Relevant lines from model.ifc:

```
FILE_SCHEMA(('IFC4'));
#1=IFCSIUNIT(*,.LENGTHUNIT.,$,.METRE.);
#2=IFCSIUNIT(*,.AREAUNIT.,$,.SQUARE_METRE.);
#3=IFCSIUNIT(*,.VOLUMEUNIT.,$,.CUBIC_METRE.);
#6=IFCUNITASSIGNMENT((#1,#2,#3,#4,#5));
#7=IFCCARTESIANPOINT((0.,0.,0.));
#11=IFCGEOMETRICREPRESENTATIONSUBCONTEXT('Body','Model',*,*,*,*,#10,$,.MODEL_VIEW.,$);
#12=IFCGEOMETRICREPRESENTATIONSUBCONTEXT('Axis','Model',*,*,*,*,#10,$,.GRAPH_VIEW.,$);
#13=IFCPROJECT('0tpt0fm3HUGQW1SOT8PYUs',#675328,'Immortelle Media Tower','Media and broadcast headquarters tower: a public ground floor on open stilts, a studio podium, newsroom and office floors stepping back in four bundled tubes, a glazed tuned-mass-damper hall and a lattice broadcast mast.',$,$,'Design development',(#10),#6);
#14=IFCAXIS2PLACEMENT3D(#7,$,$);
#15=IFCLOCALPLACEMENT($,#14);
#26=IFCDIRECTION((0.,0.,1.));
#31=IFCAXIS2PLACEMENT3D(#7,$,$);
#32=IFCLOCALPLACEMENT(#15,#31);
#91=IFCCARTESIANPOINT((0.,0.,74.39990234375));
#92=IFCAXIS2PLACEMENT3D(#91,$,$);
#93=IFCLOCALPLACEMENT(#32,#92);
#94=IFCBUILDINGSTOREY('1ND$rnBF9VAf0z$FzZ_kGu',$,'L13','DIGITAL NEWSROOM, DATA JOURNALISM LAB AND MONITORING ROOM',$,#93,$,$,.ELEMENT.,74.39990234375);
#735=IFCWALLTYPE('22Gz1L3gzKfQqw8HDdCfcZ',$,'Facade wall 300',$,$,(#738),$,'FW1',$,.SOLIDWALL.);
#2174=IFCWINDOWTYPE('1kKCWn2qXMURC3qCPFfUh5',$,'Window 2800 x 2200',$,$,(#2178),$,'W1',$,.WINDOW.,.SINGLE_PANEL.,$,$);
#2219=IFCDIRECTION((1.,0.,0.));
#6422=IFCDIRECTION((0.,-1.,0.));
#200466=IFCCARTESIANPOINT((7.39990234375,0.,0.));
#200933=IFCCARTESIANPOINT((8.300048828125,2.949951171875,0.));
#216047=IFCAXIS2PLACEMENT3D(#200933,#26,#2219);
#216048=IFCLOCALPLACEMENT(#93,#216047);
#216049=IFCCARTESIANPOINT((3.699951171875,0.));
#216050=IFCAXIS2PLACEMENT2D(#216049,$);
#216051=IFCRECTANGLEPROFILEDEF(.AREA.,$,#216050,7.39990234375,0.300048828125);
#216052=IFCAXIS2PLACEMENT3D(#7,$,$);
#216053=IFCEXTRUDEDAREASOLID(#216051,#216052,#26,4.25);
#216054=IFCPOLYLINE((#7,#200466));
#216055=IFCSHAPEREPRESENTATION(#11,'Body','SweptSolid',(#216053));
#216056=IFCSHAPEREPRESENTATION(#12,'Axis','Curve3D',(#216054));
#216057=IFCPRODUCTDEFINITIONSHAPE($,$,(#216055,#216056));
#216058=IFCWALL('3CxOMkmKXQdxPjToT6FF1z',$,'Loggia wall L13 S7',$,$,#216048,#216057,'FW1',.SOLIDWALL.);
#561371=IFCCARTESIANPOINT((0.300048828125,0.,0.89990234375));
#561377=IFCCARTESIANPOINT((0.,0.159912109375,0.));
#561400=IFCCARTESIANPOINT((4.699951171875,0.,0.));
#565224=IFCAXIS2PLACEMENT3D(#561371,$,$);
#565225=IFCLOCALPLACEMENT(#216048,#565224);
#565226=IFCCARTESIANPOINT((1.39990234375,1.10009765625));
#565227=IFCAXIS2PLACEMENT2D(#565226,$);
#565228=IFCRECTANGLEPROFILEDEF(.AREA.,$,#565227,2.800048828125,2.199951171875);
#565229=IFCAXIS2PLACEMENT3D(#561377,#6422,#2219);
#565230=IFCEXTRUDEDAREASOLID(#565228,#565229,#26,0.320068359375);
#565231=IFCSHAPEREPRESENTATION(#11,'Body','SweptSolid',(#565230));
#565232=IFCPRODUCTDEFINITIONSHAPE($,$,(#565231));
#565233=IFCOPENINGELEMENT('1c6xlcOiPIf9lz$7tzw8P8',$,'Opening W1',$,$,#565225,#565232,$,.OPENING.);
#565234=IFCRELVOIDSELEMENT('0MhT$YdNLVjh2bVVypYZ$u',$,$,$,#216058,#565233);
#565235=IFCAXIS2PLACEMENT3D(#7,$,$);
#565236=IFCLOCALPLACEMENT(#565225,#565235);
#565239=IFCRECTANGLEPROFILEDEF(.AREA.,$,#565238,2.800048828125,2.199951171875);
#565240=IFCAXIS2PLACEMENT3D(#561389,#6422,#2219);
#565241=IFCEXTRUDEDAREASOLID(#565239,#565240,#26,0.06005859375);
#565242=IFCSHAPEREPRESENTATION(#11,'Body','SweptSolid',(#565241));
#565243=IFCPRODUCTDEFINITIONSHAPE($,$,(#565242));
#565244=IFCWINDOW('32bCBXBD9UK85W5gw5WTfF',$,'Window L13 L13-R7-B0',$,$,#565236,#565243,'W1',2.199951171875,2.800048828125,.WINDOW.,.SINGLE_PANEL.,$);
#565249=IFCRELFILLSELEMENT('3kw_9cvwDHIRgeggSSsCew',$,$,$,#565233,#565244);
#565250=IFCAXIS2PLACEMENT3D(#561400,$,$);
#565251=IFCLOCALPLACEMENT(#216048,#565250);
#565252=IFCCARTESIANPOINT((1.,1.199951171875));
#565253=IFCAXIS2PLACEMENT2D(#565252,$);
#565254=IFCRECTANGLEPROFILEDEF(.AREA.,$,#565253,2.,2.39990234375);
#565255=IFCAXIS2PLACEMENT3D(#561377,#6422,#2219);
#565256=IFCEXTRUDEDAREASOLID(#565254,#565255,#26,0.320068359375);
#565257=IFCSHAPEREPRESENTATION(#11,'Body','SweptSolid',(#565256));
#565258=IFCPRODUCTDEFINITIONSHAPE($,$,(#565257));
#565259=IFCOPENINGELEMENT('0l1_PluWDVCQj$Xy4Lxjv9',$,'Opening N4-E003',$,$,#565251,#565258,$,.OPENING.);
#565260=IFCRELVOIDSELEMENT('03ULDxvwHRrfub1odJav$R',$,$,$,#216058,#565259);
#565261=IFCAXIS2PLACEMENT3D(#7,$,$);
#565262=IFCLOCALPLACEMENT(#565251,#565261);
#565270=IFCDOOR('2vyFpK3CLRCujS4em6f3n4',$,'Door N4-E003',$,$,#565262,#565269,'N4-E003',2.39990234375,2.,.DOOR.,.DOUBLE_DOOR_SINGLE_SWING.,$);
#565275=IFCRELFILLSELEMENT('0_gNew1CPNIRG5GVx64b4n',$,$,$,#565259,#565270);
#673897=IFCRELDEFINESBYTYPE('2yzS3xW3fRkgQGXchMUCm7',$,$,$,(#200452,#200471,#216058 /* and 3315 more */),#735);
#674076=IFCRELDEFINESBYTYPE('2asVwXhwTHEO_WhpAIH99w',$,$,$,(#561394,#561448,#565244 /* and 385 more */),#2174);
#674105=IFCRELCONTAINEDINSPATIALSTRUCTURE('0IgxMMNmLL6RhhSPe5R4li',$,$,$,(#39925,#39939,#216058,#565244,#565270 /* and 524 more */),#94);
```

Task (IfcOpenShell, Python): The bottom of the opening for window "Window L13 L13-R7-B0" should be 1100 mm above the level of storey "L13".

```python
import numpy as np
import ifcopenshell
import ifcopenshell.api.geometry
import ifcopenshell.geom
import ifcopenshell.util.element
import ifcopenshell.util.placement
import ifcopenshell.util.shape
import ifcopenshell.util.unit

model = ifcopenshell.open("model.ifc")
unit_scale = ifcopenshell.util.unit.calculate_unit_scale(model)

window = model.by_id(565244)
opening = window.FillsVoids[0].RelatingOpeningElement
storey = ifcopenshell.util.element.get_container(window, ifc_class="IfcBuildingStorey")
level = ifcopenshell.util.placement.get_local_placement(storey.ObjectPlacement)[2, 3]

# The opening's origin need not be at the sill, so measure its lowest point.
shape = ifcopenshell.geom.create_shape(ifcopenshell.geom.settings(), opening)
bottom = ifcopenshell.util.shape.get_shape_bottom_elevation(shape, shape.geometry) / unit_scale
dz = level + 1.1 / unit_scale - bottom

shift = np.array([0.0, 0.0, dz])
# The window is placed relative to its opening, so it follows when the opening moves.
matrix = ifcopenshell.util.placement.get_local_placement(opening.ObjectPlacement)
matrix[:3, 3] += shift
ifcopenshell.api.geometry.edit_object_placement(
    model, product=opening, matrix=matrix, is_si=False, should_transform_children=True
)

print(f"moved by {dz * unit_scale:+.3f} m")

model.write("model_edited.ifc")
```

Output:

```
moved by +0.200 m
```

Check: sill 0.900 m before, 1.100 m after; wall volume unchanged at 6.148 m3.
